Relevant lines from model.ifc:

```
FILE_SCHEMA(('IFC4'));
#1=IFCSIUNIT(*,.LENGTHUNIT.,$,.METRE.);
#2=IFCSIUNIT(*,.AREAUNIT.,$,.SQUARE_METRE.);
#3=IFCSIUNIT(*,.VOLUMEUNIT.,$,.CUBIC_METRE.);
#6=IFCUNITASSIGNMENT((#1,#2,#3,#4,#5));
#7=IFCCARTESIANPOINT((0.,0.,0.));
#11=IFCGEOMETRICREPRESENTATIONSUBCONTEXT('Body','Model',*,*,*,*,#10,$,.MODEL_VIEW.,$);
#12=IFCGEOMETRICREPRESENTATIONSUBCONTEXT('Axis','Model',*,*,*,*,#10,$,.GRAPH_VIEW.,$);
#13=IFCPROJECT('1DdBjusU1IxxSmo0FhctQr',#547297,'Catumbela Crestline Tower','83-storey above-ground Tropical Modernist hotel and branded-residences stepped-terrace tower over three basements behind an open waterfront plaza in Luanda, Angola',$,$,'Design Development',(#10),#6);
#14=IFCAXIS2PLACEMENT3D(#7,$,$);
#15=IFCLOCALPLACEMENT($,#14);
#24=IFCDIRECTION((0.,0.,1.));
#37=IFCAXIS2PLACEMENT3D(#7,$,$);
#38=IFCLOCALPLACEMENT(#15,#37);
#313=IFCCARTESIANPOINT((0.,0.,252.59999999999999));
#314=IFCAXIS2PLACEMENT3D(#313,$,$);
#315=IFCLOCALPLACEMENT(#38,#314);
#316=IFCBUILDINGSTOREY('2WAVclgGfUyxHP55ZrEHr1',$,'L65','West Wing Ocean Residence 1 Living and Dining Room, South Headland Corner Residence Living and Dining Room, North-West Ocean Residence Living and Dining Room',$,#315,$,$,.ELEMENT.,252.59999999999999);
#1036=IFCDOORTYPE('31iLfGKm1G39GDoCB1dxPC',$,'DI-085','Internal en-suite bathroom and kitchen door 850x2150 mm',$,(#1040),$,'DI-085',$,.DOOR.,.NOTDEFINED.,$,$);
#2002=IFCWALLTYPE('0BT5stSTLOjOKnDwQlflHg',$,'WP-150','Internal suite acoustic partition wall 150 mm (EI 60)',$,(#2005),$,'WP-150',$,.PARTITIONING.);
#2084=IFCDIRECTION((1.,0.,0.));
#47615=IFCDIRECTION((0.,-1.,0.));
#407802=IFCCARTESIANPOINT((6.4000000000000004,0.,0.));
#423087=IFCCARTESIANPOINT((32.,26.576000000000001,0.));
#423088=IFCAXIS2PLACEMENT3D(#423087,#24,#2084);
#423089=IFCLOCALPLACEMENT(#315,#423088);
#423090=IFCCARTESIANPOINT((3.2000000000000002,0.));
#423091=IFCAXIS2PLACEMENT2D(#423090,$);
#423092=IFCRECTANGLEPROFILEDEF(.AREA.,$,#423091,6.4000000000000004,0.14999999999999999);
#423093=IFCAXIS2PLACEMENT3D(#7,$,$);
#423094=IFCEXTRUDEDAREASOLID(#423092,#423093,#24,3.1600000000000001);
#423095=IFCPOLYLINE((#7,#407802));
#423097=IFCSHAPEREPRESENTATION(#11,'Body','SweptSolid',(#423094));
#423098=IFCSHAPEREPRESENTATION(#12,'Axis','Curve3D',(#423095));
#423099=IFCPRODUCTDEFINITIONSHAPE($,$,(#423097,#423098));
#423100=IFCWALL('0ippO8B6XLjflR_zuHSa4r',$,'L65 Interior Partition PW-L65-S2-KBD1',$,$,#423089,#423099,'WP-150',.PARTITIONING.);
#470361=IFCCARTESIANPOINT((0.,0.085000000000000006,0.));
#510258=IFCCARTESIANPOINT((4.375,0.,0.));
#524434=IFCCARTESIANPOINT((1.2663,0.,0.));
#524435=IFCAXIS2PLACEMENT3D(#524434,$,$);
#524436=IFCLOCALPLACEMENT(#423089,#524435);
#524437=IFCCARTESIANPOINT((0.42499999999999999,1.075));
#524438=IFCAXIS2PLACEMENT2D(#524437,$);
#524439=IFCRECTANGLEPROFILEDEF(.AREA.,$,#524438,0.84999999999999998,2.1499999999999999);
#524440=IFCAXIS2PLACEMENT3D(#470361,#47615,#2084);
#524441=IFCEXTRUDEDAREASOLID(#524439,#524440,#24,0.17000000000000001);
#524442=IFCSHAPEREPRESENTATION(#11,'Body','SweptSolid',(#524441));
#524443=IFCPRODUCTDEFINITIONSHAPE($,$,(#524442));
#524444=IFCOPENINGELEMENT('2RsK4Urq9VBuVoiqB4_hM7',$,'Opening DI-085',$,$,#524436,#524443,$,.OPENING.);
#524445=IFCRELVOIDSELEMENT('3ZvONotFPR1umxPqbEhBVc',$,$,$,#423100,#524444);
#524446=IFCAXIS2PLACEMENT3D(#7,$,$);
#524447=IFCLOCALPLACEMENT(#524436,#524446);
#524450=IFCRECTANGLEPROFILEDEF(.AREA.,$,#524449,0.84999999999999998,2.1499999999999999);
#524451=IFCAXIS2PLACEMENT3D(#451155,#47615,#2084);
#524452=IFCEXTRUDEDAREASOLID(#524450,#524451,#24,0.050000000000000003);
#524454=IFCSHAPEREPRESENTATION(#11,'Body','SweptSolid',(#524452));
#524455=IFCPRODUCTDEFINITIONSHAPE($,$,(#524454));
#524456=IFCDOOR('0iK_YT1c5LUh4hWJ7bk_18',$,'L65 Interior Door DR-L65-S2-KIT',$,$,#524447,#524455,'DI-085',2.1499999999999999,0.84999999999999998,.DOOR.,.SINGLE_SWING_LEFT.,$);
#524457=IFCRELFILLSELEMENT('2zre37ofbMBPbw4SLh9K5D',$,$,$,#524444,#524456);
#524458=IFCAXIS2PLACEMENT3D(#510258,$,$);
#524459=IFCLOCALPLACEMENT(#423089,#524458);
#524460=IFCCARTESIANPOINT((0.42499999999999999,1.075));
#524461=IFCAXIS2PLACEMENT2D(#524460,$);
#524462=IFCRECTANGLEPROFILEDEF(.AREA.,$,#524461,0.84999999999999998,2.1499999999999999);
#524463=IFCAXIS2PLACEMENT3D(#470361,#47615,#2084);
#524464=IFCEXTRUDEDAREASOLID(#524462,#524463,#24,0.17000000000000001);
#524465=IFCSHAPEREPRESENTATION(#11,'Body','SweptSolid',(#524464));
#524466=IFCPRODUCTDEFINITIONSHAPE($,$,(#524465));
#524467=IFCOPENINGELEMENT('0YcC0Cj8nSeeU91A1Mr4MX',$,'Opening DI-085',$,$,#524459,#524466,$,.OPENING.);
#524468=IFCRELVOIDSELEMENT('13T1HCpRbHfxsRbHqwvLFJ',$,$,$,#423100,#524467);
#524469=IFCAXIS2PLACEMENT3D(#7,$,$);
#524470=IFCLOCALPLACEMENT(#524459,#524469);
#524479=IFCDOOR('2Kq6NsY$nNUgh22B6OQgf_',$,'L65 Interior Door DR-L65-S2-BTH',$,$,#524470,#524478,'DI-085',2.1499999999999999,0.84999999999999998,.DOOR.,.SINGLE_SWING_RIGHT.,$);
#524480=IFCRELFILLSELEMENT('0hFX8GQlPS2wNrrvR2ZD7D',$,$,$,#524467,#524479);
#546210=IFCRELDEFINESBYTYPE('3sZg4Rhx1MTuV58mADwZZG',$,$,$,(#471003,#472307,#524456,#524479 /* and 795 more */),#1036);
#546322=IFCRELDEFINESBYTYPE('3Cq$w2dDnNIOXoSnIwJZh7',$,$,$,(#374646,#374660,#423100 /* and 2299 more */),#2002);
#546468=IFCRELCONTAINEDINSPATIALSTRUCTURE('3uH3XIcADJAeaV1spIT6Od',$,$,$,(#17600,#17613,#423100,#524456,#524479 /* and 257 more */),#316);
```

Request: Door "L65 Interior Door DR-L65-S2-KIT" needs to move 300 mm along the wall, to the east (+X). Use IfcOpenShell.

```python
import ifcopenshell
import ifcopenshell.api.geometry
import ifcopenshell.util.placement
import ifcopenshell.util.unit

model = ifcopenshell.open("model.ifc")
unit_scale = ifcopenshell.util.unit.calculate_unit_scale(model)

door = model.by_guid("0iK_YT1c5LUh4hWJ7bk_18")
opening = door.FillsVoids[0].RelatingOpeningElement
wall = opening.VoidsElements[0].RelatingBuildingElement

wall_matrix = ifcopenshell.util.placement.get_local_placement(wall.ObjectPlacement)
shift = wall_matrix[:3, 0] * 0.3 / unit_scale
before = ifcopenshell.util.placement.get_local_placement(door.ObjectPlacement)[:3, 3].copy()

# The door is placed relative to its opening, so it follows when the opening moves.
matrix = ifcopenshell.util.placement.get_local_placement(opening.ObjectPlacement)
matrix[:3, 3] += shift
ifcopenshell.api.geometry.edit_object_placement(
    model, product=opening, matrix=matrix, is_si=False, should_transform_children=True
)

after = ifcopenshell.util.placement.get_local_placement(door.ObjectPlacement)[:3, 3]
print("door moved by", (after - before).round(3) + 0.0)

model.write("model_edited.ifc")
```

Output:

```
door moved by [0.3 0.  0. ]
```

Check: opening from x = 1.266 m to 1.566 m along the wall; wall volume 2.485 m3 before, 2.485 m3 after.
